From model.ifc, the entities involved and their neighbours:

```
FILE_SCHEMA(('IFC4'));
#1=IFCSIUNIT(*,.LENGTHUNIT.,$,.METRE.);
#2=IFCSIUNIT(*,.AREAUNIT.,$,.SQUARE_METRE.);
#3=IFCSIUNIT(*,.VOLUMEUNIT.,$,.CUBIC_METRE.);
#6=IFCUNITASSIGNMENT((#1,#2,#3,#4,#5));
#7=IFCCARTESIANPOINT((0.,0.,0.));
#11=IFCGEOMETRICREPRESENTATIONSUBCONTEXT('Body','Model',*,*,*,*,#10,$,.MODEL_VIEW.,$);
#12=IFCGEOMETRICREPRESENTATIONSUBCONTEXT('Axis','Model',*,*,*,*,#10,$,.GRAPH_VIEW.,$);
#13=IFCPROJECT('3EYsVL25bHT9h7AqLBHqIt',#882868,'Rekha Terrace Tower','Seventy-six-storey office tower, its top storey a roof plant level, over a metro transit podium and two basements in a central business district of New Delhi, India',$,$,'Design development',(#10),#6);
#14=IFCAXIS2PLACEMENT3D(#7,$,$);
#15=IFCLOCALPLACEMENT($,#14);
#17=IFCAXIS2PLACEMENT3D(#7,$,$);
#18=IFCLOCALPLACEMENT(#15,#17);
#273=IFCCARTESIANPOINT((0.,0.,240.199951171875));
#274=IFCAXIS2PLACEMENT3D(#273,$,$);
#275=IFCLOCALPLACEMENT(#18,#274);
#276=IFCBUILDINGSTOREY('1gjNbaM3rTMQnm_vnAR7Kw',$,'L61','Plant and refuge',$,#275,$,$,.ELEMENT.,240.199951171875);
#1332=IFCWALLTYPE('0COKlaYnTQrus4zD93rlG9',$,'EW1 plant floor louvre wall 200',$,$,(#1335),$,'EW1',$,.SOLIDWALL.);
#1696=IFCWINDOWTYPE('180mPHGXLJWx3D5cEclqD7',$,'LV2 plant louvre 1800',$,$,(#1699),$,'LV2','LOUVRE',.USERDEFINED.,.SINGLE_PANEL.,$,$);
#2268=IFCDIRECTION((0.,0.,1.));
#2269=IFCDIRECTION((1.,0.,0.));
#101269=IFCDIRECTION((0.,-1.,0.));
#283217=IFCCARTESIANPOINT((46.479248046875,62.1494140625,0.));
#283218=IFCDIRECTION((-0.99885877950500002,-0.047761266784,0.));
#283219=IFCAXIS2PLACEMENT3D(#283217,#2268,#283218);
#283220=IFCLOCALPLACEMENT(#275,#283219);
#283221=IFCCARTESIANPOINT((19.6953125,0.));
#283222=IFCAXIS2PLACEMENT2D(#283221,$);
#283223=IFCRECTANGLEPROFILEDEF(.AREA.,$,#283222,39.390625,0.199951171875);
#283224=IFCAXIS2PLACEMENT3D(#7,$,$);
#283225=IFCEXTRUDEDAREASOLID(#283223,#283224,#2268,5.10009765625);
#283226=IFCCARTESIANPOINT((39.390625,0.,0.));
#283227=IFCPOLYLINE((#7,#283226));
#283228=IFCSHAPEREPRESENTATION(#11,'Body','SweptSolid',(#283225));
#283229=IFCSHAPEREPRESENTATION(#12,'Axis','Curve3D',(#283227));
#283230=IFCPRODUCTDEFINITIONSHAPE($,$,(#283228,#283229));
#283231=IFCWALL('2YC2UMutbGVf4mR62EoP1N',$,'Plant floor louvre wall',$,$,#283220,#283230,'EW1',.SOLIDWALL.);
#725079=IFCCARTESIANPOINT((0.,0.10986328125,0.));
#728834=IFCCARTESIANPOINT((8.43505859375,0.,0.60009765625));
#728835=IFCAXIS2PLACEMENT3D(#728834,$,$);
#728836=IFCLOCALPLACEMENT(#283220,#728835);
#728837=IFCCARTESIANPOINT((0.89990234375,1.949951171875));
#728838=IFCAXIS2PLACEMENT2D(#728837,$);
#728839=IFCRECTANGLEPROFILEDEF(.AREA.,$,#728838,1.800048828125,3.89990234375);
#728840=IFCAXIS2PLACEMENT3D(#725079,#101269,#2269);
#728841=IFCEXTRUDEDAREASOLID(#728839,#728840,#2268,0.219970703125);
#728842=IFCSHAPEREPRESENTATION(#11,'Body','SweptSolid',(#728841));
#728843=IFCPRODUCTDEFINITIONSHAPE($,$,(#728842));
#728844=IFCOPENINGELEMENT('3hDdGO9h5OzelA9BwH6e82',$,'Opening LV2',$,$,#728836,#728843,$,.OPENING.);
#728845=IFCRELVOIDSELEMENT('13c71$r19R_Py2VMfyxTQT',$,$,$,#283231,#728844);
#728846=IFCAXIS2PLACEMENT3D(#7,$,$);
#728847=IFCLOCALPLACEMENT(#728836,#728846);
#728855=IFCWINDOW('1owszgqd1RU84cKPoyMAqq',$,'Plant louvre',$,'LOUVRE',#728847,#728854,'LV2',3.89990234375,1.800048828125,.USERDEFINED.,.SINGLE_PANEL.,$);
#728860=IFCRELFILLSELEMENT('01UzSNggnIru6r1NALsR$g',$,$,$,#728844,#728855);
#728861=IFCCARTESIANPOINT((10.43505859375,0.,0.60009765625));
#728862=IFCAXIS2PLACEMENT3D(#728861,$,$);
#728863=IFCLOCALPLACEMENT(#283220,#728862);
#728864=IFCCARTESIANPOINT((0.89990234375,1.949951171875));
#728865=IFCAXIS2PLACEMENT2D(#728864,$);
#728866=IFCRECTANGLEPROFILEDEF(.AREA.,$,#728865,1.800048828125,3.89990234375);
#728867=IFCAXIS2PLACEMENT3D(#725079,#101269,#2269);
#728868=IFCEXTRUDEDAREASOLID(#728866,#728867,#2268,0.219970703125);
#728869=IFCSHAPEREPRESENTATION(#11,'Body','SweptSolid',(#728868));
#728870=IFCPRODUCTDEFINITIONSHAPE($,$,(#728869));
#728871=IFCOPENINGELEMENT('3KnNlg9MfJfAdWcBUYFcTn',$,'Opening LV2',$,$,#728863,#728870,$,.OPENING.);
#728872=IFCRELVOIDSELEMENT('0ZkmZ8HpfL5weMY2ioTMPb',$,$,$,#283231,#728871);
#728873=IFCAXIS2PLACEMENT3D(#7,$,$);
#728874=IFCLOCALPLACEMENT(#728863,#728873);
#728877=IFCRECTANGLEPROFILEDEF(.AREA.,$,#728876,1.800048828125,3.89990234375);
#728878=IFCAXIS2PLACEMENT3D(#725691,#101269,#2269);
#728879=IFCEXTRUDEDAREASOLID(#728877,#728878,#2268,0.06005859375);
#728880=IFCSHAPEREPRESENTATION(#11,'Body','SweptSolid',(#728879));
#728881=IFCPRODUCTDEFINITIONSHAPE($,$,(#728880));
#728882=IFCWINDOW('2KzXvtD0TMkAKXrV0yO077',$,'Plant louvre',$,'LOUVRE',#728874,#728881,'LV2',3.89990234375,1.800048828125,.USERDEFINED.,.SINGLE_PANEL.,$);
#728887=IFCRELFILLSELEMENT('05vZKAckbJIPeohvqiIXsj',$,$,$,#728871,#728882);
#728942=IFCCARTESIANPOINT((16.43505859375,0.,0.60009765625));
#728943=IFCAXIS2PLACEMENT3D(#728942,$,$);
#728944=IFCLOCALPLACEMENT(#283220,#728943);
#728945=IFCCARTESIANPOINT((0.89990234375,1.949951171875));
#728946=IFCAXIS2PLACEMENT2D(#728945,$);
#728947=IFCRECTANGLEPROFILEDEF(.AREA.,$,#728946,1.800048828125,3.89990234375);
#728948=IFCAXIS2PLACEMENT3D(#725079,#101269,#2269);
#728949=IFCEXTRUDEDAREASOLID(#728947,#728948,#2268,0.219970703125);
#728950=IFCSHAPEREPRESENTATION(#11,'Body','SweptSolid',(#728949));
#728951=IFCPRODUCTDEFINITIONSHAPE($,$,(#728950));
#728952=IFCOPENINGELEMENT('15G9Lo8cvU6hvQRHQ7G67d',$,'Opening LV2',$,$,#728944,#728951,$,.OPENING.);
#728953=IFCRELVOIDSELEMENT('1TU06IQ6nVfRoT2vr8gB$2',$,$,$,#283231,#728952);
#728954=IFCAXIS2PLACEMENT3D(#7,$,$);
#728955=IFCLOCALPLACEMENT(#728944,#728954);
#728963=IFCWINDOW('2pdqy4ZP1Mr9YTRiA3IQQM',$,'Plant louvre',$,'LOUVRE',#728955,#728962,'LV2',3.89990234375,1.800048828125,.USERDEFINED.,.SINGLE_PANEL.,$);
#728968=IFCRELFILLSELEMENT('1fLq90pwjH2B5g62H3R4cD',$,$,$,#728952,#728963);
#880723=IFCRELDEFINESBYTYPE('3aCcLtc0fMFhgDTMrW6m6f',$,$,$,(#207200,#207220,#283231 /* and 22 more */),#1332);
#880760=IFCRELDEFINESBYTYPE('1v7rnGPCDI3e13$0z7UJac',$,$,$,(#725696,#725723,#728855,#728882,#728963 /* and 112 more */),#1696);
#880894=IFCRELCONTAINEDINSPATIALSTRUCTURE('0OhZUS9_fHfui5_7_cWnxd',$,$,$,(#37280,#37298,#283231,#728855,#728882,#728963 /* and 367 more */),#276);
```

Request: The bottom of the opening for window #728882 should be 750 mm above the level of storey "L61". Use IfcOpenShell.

```python
import numpy as np
import ifcopenshell
import ifcopenshell.api.geometry
import ifcopenshell.geom
import ifcopenshell.util.element
import ifcopenshell.util.placement
import ifcopenshell.util.shape
import ifcopenshell.util.unit

model = ifcopenshell.open("model.ifc")
unit_scale = ifcopenshell.util.unit.calculate_unit_scale(model)

window = model.by_guid("2KzXvtD0TMkAKXrV0yO077")
opening = window.FillsVoids[0].RelatingOpeningElement
storey = ifcopenshell.util.element.get_container(window, ifc_class="IfcBuildingStorey")
level = ifcopenshell.util.placement.get_local_placement(storey.ObjectPlacement)[2, 3]

# The opening's origin need not be at the sill, so measure its lowest point.
shape = ifcopenshell.geom.create_shape(ifcopenshell.geom.settings(), opening)
bottom = ifcopenshell.util.shape.get_shape_bottom_elevation(shape, shape.geometry) / unit_scale
dz = level + 0.75 - bottom

shift = np.array([0.0, 0.0, dz])
# The window is placed relative to its opening, so it follows when the opening moves.
matrix = ifcopenshell.util.placement.get_local_placement(opening.ObjectPlacement)
matrix[:3, 3] += shift
ifcopenshell.api.geometry.edit_object_placement(
    model, product=opening, matrix=matrix, is_si=False, should_transform_children=True
)

print(f"moved by {dz * unit_scale:+.3f} m")

model.write("model_updated.ifc")
```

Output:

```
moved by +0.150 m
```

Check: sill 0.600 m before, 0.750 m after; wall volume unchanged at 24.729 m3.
